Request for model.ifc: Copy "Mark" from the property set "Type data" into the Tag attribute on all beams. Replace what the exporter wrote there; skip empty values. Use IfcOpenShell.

First a look at what the model holds.

```python
import ifcopenshell
import ifcopenshell.util.element

model = ifcopenshell.open("model.ifc")
print(model.schema)
beams = model.by_type("IfcBeam")
print(len(beams), "beams")
for e in beams[:8]:
    source = ifcopenshell.util.element.get_pset(e, "Type data", "Mark")
    target = e.Tag
    print(e.id(), repr(source), repr(target), sep=" | ")
```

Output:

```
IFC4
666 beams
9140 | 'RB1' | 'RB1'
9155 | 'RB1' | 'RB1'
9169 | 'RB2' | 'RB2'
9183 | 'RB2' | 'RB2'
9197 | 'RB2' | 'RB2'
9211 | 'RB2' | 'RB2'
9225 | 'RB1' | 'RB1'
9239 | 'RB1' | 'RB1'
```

```python
import ifcopenshell
import ifcopenshell.util.element

model = ifcopenshell.open("model.ifc")

count = 0
for e in model.by_type("IfcBeam"):
    value = ifcopenshell.util.element.get_pset(e, "Type data", "Mark")
    current = e.Tag
    if not value or not value.strip() or current == value:
        continue
    e.Tag = value
    count += 1

print(count, "beams updated")

model.write("model_v2.ifc")
```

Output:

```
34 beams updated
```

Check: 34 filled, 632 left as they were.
